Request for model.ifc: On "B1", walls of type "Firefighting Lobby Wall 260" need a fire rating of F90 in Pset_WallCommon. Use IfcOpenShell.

First a look at what the model holds.

```python
import ifcopenshell
import ifcopenshell.util.element

model = ifcopenshell.open("model.ifc")
print(model.schema)
storey = next(s for s in model.by_type("IfcBuildingStorey") if s.Name == "B1")
walls = [e for e in ifcopenshell.util.element.get_decomposition(storey) if e.is_a("IfcWall")]
seen = {}
for e in walls:
    element_type = ifcopenshell.util.element.get_type(e)
    key = (element_type.Name if element_type != e and element_type else None, ifcopenshell.util.element.get_pset(e, "Pset_WallCommon", "FireRating"))
    seen[key] = seen.get(key, 0) + 1
for (name, value), count in sorted(seen.items(), key=str):
    print(count, "x", name, "|", value)
```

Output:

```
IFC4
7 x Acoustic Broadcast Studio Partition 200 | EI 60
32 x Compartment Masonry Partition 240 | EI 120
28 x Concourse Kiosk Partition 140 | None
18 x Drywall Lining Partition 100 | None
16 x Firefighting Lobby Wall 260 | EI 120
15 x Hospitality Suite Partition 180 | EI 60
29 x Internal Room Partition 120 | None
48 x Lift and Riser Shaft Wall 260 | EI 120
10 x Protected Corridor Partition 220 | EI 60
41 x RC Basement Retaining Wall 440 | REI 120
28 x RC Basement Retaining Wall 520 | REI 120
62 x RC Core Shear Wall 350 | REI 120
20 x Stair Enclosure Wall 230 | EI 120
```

```python
import ifcopenshell
import ifcopenshell.api.pset
import ifcopenshell.util.element

model = ifcopenshell.open("model.ifc")

storey = next(s for s in model.by_type("IfcBuildingStorey") if s.Name == "B1")
walls = [e for e in ifcopenshell.util.element.get_decomposition(storey) if e.is_a("IfcWall")]

count = 0
for e in walls:
    element_type = ifcopenshell.util.element.get_type(e)
    if element_type in (None, e) or element_type.Name != "Firefighting Lobby Wall 260":
        continue
    # add_pset returns the element's existing set when there is one.
    pset = ifcopenshell.api.pset.add_pset(model, product=e, name="Pset_WallCommon")
    ifcopenshell.api.pset.edit_pset(model, pset=pset, properties={"FireRating": "F90"})
    count += 1

print(count, "walls updated")

model.write("model_v2.ifc")
```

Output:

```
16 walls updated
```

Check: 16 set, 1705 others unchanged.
